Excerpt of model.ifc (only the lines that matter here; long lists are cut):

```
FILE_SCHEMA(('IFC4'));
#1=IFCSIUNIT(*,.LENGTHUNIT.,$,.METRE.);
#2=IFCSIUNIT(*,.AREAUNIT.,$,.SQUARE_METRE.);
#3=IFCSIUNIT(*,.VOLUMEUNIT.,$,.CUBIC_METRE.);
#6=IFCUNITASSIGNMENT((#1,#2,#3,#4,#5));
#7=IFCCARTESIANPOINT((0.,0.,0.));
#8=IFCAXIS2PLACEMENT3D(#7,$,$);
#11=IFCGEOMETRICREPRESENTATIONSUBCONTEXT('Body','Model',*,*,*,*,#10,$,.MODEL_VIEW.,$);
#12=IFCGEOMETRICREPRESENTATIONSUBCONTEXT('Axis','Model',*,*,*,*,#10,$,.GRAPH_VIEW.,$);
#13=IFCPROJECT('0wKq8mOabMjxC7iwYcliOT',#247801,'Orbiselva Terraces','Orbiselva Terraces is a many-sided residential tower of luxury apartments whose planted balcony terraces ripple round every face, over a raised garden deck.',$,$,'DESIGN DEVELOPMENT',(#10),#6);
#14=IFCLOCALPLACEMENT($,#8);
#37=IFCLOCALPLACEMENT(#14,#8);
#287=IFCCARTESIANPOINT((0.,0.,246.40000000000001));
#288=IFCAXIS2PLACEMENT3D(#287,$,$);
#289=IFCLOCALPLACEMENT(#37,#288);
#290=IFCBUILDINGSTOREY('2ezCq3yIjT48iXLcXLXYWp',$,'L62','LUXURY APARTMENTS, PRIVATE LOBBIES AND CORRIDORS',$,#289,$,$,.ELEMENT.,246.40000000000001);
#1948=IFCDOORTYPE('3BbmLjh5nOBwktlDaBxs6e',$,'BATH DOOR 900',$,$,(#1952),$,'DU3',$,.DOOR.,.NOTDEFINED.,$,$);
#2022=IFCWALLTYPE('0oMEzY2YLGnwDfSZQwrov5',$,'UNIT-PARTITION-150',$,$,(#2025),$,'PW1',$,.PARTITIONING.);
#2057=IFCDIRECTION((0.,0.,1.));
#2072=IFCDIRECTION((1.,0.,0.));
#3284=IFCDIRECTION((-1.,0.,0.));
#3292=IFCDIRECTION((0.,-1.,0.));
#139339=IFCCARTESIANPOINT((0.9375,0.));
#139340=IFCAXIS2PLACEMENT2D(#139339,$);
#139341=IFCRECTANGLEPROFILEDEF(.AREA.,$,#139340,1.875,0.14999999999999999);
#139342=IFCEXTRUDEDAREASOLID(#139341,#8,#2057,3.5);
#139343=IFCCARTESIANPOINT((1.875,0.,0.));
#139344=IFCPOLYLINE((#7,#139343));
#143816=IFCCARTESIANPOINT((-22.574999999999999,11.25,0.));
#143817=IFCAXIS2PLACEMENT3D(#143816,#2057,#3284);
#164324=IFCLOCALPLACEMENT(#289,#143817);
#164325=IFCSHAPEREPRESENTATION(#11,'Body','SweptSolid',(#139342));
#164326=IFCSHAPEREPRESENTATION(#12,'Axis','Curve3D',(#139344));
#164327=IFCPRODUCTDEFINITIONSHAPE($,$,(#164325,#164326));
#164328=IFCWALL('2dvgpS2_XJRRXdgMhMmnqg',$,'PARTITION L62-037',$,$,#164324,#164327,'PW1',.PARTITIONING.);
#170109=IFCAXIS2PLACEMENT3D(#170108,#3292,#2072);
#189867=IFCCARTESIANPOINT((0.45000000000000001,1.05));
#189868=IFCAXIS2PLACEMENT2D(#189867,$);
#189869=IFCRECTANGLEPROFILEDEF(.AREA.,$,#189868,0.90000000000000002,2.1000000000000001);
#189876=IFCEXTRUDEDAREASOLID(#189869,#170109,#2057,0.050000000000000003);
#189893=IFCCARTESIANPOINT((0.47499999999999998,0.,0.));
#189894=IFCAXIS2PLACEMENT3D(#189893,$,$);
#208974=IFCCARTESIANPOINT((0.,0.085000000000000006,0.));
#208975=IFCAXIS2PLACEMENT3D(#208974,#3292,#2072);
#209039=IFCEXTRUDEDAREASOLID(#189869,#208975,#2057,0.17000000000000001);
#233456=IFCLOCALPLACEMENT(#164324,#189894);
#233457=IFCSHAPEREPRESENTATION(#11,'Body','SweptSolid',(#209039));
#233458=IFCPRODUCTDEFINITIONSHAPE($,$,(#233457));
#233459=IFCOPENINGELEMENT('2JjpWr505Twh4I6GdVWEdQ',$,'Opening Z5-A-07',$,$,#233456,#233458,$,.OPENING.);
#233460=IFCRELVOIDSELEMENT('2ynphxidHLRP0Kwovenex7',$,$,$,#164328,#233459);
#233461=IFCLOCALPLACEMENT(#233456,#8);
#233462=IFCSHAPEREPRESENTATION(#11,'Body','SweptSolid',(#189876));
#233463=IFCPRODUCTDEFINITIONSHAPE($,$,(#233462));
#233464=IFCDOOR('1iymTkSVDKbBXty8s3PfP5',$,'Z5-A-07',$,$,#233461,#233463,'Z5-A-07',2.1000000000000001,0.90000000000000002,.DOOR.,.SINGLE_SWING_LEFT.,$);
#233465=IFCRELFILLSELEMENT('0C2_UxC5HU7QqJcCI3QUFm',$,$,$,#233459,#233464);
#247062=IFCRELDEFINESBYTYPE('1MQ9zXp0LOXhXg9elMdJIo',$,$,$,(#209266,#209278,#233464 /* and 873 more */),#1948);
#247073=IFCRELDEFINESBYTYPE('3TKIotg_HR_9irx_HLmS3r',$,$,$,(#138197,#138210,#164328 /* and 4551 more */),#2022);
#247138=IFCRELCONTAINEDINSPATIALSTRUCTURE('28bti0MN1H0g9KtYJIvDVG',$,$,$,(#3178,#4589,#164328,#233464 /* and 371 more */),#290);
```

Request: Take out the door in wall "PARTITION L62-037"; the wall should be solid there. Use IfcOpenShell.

```python
import ifcopenshell
import ifcopenshell.api.feature
import ifcopenshell.api.root
import ifcopenshell.geom
import ifcopenshell.util.shape

model = ifcopenshell.open("model.ifc")
settings = ifcopenshell.geom.settings()


def volume(element):
    """Net volume in cubic metres, openings subtracted."""
    shape = ifcopenshell.geom.create_shape(settings, element)
    return ifcopenshell.util.shape.get_volume(shape.geometry)


door = model.by_guid("1iymTkSVDKbBXty8s3PfP5")
opening = door.FillsVoids[0].RelatingOpeningElement
wall = opening.VoidsElements[0].RelatingBuildingElement
before = volume(wall)

ifcopenshell.api.root.remove_product(model, product=door)
ifcopenshell.api.feature.remove_feature(model, feature=opening)

after = volume(wall)

print(f"wall volume {before:.3f} -> {after:.3f} m3")

model.write("model-out.ifc")
```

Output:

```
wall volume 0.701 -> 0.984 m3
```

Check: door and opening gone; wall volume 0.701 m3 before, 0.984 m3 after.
